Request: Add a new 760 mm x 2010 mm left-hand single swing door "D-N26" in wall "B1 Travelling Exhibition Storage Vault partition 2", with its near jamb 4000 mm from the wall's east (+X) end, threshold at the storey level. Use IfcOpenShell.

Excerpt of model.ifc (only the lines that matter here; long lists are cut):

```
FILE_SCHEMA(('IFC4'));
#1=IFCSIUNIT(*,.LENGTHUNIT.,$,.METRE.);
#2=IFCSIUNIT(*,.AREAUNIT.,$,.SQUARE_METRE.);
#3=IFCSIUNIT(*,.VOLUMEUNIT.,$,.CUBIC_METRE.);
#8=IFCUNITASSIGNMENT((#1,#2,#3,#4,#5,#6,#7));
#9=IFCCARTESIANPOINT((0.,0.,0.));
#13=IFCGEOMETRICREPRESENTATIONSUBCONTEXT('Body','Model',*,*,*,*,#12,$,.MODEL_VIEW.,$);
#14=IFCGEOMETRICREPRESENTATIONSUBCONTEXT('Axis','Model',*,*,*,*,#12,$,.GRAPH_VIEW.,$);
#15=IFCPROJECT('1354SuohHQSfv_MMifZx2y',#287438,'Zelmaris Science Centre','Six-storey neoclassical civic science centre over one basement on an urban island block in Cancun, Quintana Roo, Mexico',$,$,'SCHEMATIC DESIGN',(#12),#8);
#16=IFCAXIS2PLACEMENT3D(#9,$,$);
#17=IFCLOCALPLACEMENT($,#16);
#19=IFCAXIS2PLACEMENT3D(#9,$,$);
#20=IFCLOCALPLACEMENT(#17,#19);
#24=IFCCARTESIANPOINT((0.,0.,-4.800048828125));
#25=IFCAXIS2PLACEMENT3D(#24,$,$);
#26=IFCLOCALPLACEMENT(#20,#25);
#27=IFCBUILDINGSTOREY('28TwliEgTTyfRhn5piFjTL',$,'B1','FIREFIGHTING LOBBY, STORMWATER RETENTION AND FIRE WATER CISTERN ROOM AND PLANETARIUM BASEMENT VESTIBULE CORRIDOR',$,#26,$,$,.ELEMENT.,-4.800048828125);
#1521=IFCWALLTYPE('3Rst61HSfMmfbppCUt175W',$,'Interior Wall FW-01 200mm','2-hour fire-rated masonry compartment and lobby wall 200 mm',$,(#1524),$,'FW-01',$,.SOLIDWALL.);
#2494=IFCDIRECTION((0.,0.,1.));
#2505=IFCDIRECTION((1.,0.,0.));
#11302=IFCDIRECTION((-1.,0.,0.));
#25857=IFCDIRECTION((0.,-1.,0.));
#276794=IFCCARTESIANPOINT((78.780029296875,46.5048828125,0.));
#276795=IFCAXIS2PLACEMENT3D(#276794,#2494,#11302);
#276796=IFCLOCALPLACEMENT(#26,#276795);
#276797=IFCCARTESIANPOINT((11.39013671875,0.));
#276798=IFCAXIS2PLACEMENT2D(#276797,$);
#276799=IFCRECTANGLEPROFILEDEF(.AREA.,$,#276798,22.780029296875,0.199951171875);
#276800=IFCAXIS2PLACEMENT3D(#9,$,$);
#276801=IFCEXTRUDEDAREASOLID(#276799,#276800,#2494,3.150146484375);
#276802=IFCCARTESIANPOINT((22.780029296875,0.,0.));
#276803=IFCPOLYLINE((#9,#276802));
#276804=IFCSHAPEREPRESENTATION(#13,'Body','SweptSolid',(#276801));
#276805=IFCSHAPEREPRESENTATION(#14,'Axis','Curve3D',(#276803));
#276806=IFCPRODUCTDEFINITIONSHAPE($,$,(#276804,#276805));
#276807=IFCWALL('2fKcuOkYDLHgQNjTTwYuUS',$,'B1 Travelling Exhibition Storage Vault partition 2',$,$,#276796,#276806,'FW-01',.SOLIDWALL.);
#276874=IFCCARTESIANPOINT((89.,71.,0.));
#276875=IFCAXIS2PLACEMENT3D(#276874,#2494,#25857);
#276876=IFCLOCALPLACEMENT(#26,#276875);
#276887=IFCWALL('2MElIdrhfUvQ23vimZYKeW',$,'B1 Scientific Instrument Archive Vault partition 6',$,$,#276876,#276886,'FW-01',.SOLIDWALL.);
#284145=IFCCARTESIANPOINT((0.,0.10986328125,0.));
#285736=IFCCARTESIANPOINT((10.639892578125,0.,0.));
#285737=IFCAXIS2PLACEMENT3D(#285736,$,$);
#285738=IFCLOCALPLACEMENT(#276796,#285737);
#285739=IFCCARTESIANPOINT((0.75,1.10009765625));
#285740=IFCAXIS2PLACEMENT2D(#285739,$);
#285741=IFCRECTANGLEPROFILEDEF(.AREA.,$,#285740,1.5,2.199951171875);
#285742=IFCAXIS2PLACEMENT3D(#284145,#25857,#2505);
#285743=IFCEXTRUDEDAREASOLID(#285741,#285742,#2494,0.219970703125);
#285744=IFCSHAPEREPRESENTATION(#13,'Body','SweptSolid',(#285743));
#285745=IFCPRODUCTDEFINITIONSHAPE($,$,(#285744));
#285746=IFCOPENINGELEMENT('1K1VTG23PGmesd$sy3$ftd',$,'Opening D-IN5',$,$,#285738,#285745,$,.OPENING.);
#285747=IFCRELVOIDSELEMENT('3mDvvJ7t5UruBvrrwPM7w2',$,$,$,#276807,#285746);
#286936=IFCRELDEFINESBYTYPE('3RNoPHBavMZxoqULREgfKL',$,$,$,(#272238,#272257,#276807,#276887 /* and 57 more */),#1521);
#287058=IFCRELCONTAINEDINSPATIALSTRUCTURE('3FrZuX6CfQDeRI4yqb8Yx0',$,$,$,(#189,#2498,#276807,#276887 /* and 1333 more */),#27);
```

```python
import numpy as np
import ifcopenshell
import ifcopenshell.api.feature
import ifcopenshell.api.geometry
import ifcopenshell.api.root
import ifcopenshell.api.spatial
import ifcopenshell.geom
import ifcopenshell.util.element
import ifcopenshell.util.placement
import ifcopenshell.util.representation
import ifcopenshell.util.shape
import ifcopenshell.util.unit

model = ifcopenshell.open("model.ifc")
unit_scale = ifcopenshell.util.unit.calculate_unit_scale(model)
settings = ifcopenshell.geom.settings()


def volume(element):
    """Net volume in cubic metres, openings subtracted."""
    shape = ifcopenshell.geom.create_shape(settings, element)
    return ifcopenshell.util.shape.get_volume(shape.geometry)


wall = model.by_id(276807)
storey = ifcopenshell.util.element.get_container(wall, ifc_class="IfcBuildingStorey")
context = ifcopenshell.util.representation.get_context(model, "Model", "Body", "MODEL_VIEW")
before = volume(wall)

width, height, from_end, sill = 0.76, 2.01, 4, 0.0  # metres

# The wall runs along its own X axis, and the end named is its -X end.
wall_shape = ifcopenshell.geom.create_shape(settings, wall)
x, y, z = ifcopenshell.util.shape.get_vertices(wall_shape.geometry).T
start = x.min() + from_end
face, thickness = float(y.min()), float(y.max() - y.min())
wall_matrix = ifcopenshell.util.placement.get_local_placement(wall.ObjectPlacement)
level = ifcopenshell.util.placement.get_local_placement(storey.ObjectPlacement)[2, 3]


def in_wall(x, y):
    """Placement at x, y metres in the wall's axes, at sill height."""
    matrix = wall_matrix.copy()
    matrix[:, 3] = wall_matrix @ np.array([x / unit_scale, y / unit_scale, 0.0, 1.0])
    matrix[2, 3] = level + sill / unit_scale
    return matrix


# Opening: a box that overshoots both wall faces by 50 mm.
opening = ifcopenshell.api.root.create_entity(model, ifc_class="IfcOpeningElement", predefined_type="OPENING")
box = ifcopenshell.api.geometry.add_wall_representation(
    model, context=context, length=width, height=height, thickness=thickness + 0.1
)
ifcopenshell.api.geometry.assign_representation(model, product=opening, representation=box)
ifcopenshell.api.geometry.edit_object_placement(model, product=opening, matrix=in_wall(start, face - 0.05), is_si=False)
ifcopenshell.api.feature.add_feature(model, feature=opening, element=wall)

door = ifcopenshell.api.root.create_entity(model, ifc_class="IfcDoor", name="D-N26", predefined_type="DOOR")
door.OverallWidth, door.OverallHeight = width / unit_scale, height / unit_scale
door.OperationType = "SINGLE_SWING_LEFT"
body = ifcopenshell.api.geometry.add_door_representation(
    model,
    context=context,
    overall_width=door.OverallWidth,
    overall_height=door.OverallHeight,
    operation_type="SINGLE_SWING_LEFT",
    lining_properties={"LiningDepth": thickness / unit_scale, "ThresholdDepth": thickness / unit_scale},
)
ifcopenshell.api.geometry.assign_representation(model, product=door, representation=body)
ifcopenshell.api.spatial.assign_container(model, products=[door], relating_structure=storey)
ifcopenshell.api.feature.add_filling(model, opening=opening, element=door)

# The lining spans the wall, so the door starts at the wall face.
ifcopenshell.api.geometry.edit_object_placement(model, product=door, matrix=in_wall(start, face), is_si=False)

after = volume(wall)

print(f"wall volume {before:.3f} -> {after:.3f} m3")

model.write("model_edited.ifc")
```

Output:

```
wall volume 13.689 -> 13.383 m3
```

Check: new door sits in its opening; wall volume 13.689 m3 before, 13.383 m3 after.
